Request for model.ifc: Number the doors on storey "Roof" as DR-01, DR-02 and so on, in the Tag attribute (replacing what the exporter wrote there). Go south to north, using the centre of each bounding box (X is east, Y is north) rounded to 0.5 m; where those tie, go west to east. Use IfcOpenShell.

First a look at what the model holds.

```python
import ifcopenshell
import ifcopenshell.util.element
import ifcopenshell.util.placement

model = ifcopenshell.open("model.ifc")
print(model.schema)
storey = next(s for s in model.by_type("IfcBuildingStorey") if s.Name == "Roof")
doors = [e for e in ifcopenshell.util.element.get_decomposition(storey) if e.is_a("IfcDoor")]
for e in sorted(doors, key=lambda e: e.id()):
    origin = ifcopenshell.util.placement.get_local_placement(e.ObjectPlacement)[:3, 3]
    print(e.id(), e.Tag, e.Name, origin.round(2) + 0.0, sep=" | ")
```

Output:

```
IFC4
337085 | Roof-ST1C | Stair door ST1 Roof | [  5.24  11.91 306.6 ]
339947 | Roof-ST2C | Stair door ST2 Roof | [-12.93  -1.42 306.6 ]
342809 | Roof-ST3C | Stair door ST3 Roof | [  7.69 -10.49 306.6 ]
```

```python
import ifcopenshell
import ifcopenshell.geom
import ifcopenshell.util.element
import ifcopenshell.util.shape

model = ifcopenshell.open("model.ifc")
settings = ifcopenshell.geom.settings()
settings.set("use-world-coords", True)


def centre(element):
    shape = ifcopenshell.geom.create_shape(settings, element)
    return ifcopenshell.util.shape.get_bbox_centroid(shape.geometry)


storey = next(s for s in model.by_type("IfcBuildingStorey") if s.Name == "Roof")
doors = [e for e in ifcopenshell.util.element.get_decomposition(storey) if e.is_a("IfcDoor")]

# Insertion points can sit at a corner or the storey origin, so sort by the geometry (in metres).
centres = {e: centre(e) for e in doors}
doors.sort(key=lambda e: (round(centres[e][1] / 0.5), centres[e][0]))

for i, e in enumerate(doors, start=1):
    number = f"DR-{i:02d}"
    e.Tag = number
    print(e.id(), number)

model.write("model_edited.ifc")
```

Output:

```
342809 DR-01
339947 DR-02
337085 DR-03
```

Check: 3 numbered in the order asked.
